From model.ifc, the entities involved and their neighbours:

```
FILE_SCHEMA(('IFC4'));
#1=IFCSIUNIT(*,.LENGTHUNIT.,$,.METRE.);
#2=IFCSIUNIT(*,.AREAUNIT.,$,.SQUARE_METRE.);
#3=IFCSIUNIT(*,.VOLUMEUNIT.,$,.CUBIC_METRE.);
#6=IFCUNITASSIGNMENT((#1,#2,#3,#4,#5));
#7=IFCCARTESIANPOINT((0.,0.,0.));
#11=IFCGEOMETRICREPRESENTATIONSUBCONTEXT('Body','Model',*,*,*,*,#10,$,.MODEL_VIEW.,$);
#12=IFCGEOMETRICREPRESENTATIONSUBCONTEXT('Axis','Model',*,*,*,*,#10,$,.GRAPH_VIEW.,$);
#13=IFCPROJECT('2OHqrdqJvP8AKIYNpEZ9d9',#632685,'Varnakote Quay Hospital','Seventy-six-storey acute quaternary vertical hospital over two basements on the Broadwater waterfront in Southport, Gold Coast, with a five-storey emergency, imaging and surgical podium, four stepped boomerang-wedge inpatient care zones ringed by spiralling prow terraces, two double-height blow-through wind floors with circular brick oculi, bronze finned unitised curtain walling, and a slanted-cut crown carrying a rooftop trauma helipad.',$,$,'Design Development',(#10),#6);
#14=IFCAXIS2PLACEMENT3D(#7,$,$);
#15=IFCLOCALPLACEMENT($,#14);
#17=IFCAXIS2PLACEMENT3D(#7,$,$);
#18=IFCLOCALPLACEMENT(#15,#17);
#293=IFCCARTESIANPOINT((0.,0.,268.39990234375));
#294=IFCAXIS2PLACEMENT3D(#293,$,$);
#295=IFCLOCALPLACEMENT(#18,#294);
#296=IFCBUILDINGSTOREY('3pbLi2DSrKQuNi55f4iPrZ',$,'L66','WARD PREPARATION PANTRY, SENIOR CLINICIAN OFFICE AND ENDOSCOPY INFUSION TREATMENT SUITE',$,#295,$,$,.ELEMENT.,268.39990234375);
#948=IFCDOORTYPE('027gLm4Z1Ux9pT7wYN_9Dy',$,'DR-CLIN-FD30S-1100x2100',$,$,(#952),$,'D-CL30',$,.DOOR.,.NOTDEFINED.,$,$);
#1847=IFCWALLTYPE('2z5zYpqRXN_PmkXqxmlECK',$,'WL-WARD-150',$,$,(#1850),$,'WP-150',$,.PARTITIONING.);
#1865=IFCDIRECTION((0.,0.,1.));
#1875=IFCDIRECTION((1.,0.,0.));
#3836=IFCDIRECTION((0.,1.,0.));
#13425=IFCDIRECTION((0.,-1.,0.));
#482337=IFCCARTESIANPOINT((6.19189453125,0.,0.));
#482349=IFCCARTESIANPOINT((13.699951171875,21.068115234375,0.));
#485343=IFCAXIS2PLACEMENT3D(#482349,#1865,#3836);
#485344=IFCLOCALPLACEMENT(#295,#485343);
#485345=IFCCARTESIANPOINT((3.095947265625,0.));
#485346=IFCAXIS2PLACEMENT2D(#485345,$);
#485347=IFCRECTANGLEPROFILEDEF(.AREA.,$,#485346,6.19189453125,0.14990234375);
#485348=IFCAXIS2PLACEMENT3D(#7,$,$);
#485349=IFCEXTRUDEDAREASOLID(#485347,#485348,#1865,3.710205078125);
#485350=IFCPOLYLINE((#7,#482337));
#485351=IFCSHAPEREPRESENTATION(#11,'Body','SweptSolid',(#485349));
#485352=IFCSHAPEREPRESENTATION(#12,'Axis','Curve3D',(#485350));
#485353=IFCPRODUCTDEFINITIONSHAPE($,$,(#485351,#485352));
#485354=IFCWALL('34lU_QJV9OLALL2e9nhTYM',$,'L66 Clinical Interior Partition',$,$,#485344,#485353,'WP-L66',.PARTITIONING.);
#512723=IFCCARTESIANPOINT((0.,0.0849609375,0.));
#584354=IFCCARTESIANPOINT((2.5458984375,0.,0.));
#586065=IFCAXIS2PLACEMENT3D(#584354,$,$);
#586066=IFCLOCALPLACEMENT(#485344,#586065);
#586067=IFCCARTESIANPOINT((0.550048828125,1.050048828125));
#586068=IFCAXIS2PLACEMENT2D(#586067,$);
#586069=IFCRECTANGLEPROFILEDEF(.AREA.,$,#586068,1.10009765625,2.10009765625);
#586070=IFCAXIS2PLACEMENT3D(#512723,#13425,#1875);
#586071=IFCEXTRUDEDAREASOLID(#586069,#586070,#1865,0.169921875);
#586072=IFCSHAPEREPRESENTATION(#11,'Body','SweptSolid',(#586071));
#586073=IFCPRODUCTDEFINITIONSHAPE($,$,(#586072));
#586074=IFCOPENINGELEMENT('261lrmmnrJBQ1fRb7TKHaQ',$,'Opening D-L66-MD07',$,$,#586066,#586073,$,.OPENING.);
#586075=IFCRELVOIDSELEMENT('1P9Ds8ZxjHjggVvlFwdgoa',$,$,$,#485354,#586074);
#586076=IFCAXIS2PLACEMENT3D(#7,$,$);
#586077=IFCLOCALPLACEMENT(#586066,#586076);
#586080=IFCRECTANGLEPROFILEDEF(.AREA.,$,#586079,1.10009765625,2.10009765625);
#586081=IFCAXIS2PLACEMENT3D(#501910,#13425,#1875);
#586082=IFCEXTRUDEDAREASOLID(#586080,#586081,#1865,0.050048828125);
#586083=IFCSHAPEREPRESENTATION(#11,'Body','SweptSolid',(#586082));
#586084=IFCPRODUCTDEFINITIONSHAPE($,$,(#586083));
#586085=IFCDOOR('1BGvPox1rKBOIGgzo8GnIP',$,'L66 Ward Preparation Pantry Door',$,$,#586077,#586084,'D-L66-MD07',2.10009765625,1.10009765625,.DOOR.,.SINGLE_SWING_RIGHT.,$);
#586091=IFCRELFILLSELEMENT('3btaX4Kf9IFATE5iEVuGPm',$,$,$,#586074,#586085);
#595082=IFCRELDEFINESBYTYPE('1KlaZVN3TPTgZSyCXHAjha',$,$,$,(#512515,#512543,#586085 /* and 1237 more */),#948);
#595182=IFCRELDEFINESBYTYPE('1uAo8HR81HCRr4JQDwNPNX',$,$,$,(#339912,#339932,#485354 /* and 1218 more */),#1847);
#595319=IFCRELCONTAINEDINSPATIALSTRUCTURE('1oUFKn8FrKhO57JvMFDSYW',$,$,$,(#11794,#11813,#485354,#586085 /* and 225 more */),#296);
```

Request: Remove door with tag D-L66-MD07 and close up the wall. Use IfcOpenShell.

```python
import ifcopenshell
import ifcopenshell.api.feature
import ifcopenshell.api.root
import ifcopenshell.geom
import ifcopenshell.util.shape

model = ifcopenshell.open("model.ifc")
settings = ifcopenshell.geom.settings()


def volume(element):
    """Net volume in cubic metres, openings subtracted."""
    shape = ifcopenshell.geom.create_shape(settings, element)
    return ifcopenshell.util.shape.get_volume(shape.geometry)


door = model.by_guid("1BGvPox1rKBOIGgzo8GnIP")
opening = door.FillsVoids[0].RelatingOpeningElement
wall = opening.VoidsElements[0].RelatingBuildingElement
before = volume(wall)

ifcopenshell.api.root.remove_product(model, product=door)
ifcopenshell.api.feature.remove_feature(model, feature=opening)

after = volume(wall)

print(f"wall volume {before:.3f} -> {after:.3f} m3")

model.write("model_v2.ifc")
```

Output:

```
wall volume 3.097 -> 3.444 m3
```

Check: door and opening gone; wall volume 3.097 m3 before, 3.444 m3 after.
